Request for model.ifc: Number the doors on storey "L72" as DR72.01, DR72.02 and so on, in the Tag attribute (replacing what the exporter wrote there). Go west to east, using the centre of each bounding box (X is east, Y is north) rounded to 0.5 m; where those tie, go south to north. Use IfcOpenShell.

First a look at what the model holds.

```python
import ifcopenshell
import ifcopenshell.util.element
import ifcopenshell.util.placement

model = ifcopenshell.open("model.ifc")
print(model.schema)
storey = next(s for s in model.by_type("IfcBuildingStorey") if s.Name == "L72")
doors = [e for e in ifcopenshell.util.element.get_decomposition(storey) if e.is_a("IfcDoor")]
for e in sorted(doors, key=lambda e: e.id()):
    origin = ifcopenshell.util.placement.get_local_placement(e.ObjectPlacement)[:3, 3]
    print(e.id(), e.Tag, e.Name, origin.round(2) + 0.0, sep=" | ")
```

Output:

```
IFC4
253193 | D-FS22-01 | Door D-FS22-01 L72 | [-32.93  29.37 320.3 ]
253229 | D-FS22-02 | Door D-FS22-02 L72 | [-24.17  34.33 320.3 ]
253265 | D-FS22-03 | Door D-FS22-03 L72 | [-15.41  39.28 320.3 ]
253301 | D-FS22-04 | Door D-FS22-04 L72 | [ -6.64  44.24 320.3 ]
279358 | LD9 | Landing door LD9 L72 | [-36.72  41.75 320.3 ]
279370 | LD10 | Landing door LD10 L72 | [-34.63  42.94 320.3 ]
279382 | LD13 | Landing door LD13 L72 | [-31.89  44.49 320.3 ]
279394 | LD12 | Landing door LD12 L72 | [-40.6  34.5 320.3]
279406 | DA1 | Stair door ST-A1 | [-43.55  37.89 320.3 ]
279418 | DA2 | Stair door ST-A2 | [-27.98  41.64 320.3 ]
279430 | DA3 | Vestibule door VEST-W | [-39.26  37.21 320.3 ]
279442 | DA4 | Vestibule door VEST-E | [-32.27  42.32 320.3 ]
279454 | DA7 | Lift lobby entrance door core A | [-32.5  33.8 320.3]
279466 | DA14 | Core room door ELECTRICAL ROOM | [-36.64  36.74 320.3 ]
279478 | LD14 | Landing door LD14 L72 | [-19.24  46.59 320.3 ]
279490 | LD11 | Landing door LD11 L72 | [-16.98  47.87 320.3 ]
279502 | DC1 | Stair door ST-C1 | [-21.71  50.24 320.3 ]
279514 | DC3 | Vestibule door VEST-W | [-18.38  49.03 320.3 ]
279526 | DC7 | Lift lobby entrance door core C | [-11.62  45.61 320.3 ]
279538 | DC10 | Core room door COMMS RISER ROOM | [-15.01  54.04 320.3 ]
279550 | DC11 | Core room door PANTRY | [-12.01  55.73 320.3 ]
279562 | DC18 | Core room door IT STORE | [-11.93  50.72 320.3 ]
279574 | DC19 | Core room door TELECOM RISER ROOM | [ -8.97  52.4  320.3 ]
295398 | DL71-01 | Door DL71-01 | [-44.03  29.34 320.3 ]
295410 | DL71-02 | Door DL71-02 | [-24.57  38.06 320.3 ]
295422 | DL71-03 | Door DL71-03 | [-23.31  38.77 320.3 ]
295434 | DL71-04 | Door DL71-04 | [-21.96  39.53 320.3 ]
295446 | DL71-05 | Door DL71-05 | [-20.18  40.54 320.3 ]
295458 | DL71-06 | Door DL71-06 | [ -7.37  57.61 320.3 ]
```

```python
import ifcopenshell
import ifcopenshell.geom
import ifcopenshell.util.element
import ifcopenshell.util.shape

model = ifcopenshell.open("model.ifc")
settings = ifcopenshell.geom.settings()
settings.set("use-world-coords", True)


def centre(element):
    shape = ifcopenshell.geom.create_shape(settings, element)
    return ifcopenshell.util.shape.get_bbox_centroid(shape.geometry)


storey = next(s for s in model.by_type("IfcBuildingStorey") if s.Name == "L72")
doors = [e for e in ifcopenshell.util.element.get_decomposition(storey) if e.is_a("IfcDoor")]

# Insertion points can sit at a corner or the storey origin, so sort by the geometry (in metres).
centres = {e: centre(e) for e in doors}
doors.sort(key=lambda e: (round(centres[e][0] / 0.5), centres[e][1]))

for i, e in enumerate(doors, start=1):
    number = f"DR72.{i:02d}"
    e.Tag = number
    print(e.id(), number)

model.write("model_rev.ifc")
```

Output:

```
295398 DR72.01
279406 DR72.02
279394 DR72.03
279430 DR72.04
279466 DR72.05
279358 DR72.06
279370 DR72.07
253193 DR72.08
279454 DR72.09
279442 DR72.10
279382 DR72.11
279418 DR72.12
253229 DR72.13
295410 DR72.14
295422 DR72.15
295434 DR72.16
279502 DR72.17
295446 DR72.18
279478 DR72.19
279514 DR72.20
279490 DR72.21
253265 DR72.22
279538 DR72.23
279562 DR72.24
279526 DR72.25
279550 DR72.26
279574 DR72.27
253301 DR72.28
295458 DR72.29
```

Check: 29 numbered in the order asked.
